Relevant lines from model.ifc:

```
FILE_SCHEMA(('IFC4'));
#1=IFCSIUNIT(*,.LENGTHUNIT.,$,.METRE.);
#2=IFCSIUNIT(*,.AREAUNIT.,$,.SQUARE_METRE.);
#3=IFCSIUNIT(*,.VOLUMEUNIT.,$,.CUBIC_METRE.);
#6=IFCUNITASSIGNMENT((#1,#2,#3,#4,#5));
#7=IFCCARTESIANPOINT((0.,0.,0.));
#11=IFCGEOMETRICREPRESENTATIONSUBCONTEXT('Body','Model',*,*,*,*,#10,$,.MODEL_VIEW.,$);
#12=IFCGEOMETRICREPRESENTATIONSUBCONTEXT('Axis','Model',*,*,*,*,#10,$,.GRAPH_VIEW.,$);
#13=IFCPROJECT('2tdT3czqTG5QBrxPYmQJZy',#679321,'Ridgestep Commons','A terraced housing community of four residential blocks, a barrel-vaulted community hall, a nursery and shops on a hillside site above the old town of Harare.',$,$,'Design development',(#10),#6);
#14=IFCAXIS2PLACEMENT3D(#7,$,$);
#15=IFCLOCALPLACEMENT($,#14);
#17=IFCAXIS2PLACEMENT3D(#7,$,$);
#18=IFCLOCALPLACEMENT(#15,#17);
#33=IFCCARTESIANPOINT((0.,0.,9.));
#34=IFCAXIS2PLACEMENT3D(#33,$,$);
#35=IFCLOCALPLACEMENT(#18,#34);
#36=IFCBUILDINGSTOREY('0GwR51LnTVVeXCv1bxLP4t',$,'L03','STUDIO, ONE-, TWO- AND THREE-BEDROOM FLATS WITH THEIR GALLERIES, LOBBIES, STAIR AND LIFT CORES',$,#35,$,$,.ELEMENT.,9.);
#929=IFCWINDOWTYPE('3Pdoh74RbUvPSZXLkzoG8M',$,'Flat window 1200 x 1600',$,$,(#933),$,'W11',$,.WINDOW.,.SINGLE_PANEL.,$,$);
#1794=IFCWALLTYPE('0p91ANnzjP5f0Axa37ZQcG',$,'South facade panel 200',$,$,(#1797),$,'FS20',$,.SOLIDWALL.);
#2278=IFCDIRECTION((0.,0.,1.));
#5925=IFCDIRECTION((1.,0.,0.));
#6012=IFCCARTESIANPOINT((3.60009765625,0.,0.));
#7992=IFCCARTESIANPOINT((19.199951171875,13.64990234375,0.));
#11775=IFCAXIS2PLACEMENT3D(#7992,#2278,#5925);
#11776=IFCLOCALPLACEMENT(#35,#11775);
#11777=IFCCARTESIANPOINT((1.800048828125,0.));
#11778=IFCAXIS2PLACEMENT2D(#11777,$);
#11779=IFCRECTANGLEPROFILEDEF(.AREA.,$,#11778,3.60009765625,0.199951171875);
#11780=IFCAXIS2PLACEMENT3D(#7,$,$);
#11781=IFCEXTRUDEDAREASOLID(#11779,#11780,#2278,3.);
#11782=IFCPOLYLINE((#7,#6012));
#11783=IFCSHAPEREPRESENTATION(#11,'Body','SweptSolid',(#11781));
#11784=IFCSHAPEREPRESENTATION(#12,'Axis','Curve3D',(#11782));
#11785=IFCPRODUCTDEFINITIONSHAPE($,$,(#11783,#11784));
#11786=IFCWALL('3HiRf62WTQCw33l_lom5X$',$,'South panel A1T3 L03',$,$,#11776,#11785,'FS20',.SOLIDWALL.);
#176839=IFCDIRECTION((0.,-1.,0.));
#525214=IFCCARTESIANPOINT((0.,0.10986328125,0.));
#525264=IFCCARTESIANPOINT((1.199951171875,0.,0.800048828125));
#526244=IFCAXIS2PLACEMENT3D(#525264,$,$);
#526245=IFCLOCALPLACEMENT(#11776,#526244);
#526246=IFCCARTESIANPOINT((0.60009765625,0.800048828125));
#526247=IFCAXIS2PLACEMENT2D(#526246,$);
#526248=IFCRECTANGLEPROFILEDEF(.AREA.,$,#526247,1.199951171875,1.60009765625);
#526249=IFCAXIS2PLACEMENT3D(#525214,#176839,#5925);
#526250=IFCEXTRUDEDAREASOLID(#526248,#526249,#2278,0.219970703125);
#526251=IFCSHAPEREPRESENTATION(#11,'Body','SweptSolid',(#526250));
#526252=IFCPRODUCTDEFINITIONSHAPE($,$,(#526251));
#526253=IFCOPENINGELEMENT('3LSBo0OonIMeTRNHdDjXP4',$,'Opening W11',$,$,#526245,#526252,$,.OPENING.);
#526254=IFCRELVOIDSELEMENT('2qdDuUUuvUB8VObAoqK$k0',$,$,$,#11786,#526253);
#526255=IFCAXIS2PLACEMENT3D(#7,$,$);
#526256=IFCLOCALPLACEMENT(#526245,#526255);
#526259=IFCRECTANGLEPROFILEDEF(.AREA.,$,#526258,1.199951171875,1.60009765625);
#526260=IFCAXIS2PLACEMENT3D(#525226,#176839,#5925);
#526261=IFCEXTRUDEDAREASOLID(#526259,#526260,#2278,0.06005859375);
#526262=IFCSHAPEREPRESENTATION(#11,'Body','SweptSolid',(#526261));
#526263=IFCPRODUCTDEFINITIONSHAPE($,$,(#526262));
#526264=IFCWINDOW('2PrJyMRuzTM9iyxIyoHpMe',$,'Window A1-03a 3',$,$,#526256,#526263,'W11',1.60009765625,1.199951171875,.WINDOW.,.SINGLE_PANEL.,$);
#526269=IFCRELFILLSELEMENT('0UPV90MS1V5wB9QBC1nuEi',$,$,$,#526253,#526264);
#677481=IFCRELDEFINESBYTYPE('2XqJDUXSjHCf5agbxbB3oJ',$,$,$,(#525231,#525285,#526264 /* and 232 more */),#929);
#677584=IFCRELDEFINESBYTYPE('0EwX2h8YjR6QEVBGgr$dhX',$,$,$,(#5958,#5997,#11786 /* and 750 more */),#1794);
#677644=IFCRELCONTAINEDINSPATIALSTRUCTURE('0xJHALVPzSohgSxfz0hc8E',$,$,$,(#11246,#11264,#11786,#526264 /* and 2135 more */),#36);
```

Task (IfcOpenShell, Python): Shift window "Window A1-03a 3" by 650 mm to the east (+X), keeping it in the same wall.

```python
import ifcopenshell
import ifcopenshell.api.geometry
import ifcopenshell.util.placement

model = ifcopenshell.open("model.ifc")

window = model.by_guid("2PrJyMRuzTM9iyxIyoHpMe")
opening = window.FillsVoids[0].RelatingOpeningElement
wall = opening.VoidsElements[0].RelatingBuildingElement

wall_matrix = ifcopenshell.util.placement.get_local_placement(wall.ObjectPlacement)
shift = wall_matrix[:3, 0] * 0.65
before = ifcopenshell.util.placement.get_local_placement(window.ObjectPlacement)[:3, 3].copy()

# The window is placed relative to its opening, so it follows when the opening moves.
matrix = ifcopenshell.util.placement.get_local_placement(opening.ObjectPlacement)
matrix[:3, 3] += shift
ifcopenshell.api.geometry.edit_object_placement(
    model, product=opening, matrix=matrix, is_si=False, should_transform_children=True
)

after = ifcopenshell.util.placement.get_local_placement(window.ObjectPlacement)[:3, 3]
print("window moved by", (after - before).round(3) + 0.0)

model.write("model_rev.ifc")
```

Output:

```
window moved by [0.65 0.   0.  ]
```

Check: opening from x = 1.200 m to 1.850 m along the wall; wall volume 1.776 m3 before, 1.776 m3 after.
